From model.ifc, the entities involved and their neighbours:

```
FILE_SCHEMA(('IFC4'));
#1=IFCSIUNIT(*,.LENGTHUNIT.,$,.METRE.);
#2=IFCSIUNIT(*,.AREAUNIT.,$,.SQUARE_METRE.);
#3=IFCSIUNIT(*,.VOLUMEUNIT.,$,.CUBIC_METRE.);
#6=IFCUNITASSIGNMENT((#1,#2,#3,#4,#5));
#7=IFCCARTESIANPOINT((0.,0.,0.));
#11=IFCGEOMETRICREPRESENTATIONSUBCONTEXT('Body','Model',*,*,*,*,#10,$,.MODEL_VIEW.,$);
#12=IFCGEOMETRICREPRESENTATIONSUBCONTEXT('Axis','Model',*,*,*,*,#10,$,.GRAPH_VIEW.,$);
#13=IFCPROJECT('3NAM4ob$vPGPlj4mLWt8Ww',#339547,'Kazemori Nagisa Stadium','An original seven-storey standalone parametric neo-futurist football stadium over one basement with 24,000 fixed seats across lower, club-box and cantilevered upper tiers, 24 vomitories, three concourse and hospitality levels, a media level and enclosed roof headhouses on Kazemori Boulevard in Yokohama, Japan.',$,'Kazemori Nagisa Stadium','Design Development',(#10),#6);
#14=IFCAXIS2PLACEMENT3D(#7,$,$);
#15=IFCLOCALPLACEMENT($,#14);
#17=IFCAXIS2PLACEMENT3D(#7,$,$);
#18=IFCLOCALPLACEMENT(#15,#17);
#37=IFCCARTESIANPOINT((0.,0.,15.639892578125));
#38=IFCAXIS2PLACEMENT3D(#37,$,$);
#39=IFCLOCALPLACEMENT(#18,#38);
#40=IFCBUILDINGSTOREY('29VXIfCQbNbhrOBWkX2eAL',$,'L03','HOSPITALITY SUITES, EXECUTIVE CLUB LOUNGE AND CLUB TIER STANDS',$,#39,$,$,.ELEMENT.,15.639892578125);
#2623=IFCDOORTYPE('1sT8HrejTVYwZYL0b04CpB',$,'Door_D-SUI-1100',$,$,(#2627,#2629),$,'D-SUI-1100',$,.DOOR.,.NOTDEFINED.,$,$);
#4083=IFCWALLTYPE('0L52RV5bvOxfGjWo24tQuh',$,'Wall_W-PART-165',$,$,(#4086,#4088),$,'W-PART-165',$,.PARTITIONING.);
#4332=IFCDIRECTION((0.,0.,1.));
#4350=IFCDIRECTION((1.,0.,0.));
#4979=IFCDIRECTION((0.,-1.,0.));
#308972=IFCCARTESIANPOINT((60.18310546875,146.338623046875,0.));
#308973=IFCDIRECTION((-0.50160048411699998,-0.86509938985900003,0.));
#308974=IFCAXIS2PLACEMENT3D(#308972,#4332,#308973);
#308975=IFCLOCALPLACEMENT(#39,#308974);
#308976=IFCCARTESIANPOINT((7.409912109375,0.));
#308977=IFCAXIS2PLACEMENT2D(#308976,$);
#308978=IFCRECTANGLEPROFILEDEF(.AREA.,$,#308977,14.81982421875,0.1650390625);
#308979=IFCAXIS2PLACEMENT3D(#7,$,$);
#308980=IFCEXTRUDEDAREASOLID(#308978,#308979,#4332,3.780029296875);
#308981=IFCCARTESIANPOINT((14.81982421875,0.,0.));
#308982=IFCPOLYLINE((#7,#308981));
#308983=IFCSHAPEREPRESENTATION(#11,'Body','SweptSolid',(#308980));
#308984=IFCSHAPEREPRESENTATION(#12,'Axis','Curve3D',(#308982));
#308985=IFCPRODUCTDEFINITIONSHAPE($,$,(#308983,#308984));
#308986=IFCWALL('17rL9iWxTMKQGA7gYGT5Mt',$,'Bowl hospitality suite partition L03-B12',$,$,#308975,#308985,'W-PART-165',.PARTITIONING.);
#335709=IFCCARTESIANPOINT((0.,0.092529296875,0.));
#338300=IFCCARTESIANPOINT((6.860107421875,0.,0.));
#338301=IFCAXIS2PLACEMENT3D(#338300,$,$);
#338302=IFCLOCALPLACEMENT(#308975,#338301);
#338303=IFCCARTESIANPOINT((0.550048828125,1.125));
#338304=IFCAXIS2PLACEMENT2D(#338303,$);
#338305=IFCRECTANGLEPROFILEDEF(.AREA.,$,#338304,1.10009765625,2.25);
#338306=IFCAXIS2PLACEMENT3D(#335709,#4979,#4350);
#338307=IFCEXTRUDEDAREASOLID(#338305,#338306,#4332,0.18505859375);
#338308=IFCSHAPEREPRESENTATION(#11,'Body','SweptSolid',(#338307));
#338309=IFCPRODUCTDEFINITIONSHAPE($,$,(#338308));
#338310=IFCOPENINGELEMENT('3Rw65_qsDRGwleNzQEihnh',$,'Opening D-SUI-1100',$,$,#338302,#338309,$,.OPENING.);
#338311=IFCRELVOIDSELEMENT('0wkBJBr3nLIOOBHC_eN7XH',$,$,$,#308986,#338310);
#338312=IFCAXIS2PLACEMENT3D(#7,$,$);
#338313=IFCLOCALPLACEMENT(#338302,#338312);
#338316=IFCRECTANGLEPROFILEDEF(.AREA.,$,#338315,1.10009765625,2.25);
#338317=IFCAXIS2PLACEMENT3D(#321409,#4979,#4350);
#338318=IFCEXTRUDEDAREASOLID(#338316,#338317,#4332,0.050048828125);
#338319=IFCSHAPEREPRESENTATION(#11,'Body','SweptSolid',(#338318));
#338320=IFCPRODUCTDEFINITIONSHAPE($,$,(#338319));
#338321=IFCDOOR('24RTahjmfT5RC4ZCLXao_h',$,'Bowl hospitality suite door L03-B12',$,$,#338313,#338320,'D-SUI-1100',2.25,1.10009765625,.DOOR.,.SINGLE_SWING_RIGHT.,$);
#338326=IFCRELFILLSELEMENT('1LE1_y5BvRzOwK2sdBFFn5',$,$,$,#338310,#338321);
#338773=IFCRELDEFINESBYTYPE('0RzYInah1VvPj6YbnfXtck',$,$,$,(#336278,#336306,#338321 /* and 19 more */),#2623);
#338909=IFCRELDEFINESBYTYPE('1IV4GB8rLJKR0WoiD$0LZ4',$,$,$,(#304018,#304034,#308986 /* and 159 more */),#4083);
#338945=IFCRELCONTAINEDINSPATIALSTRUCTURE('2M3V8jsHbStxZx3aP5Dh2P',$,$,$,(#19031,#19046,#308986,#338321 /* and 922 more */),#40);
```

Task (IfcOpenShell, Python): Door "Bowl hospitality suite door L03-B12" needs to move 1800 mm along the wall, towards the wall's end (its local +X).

```python
import ifcopenshell
import ifcopenshell.api.geometry
import ifcopenshell.util.placement
import ifcopenshell.util.unit

model = ifcopenshell.open("model.ifc")
unit_scale = ifcopenshell.util.unit.calculate_unit_scale(model)

door = model.by_id(338321)
opening = door.FillsVoids[0].RelatingOpeningElement
wall = opening.VoidsElements[0].RelatingBuildingElement

wall_matrix = ifcopenshell.util.placement.get_local_placement(wall.ObjectPlacement)
shift = wall_matrix[:3, 0] * 1.8 / unit_scale
before = ifcopenshell.util.placement.get_local_placement(door.ObjectPlacement)[:3, 3].copy()

# The door is placed relative to its opening, so it follows when the opening moves.
matrix = ifcopenshell.util.placement.get_local_placement(opening.ObjectPlacement)
matrix[:3, 3] += shift
ifcopenshell.api.geometry.edit_object_placement(
    model, product=opening, matrix=matrix, is_si=False, should_transform_children=True
)

after = ifcopenshell.util.placement.get_local_placement(door.ObjectPlacement)[:3, 3]
print("door moved by", (after - before).round(3) + 0.0)

model.write("model-out.ifc")
```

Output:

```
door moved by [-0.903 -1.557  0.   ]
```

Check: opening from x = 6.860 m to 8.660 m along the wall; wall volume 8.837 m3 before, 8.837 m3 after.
